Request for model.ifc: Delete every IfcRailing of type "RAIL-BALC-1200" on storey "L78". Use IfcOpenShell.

First a look at what the model holds.

```python
import ifcopenshell
import ifcopenshell.util.element

model = ifcopenshell.open("model.ifc")
print(model.schema)
storey = next(s for s in model.by_type("IfcBuildingStorey") if s.Name == "L78")
railings = [e for e in ifcopenshell.util.element.get_decomposition(storey) if e.is_a("IfcRailing")]
seen = {}
for e in railings:
    element_type = ifcopenshell.util.element.get_type(e)
    name = element_type.Name if element_type not in (None, e) else None
    seen[name] = seen.get(name, 0) + 1
for name, count in sorted(seen.items(), key=str):
    print(count, "x", name)
```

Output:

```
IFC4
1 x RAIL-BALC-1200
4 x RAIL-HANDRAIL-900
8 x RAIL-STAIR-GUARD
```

```python
import ifcopenshell
import ifcopenshell.api.root
import ifcopenshell.util.element

model = ifcopenshell.open("model.ifc")

storey = next(s for s in model.by_type("IfcBuildingStorey") if s.Name == "L78")
railings = [e for e in ifcopenshell.util.element.get_decomposition(storey) if e.is_a("IfcRailing")]
targets = [e for e in railings if (t := ifcopenshell.util.element.get_type(e)) not in (None, e) and t.Name == "RAIL-BALC-1200"]

for e in targets:
    ifcopenshell.api.root.remove_product(model, product=e)
print(len(targets), "removed")

model.write("model_v2.ifc")
```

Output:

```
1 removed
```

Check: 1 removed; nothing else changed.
